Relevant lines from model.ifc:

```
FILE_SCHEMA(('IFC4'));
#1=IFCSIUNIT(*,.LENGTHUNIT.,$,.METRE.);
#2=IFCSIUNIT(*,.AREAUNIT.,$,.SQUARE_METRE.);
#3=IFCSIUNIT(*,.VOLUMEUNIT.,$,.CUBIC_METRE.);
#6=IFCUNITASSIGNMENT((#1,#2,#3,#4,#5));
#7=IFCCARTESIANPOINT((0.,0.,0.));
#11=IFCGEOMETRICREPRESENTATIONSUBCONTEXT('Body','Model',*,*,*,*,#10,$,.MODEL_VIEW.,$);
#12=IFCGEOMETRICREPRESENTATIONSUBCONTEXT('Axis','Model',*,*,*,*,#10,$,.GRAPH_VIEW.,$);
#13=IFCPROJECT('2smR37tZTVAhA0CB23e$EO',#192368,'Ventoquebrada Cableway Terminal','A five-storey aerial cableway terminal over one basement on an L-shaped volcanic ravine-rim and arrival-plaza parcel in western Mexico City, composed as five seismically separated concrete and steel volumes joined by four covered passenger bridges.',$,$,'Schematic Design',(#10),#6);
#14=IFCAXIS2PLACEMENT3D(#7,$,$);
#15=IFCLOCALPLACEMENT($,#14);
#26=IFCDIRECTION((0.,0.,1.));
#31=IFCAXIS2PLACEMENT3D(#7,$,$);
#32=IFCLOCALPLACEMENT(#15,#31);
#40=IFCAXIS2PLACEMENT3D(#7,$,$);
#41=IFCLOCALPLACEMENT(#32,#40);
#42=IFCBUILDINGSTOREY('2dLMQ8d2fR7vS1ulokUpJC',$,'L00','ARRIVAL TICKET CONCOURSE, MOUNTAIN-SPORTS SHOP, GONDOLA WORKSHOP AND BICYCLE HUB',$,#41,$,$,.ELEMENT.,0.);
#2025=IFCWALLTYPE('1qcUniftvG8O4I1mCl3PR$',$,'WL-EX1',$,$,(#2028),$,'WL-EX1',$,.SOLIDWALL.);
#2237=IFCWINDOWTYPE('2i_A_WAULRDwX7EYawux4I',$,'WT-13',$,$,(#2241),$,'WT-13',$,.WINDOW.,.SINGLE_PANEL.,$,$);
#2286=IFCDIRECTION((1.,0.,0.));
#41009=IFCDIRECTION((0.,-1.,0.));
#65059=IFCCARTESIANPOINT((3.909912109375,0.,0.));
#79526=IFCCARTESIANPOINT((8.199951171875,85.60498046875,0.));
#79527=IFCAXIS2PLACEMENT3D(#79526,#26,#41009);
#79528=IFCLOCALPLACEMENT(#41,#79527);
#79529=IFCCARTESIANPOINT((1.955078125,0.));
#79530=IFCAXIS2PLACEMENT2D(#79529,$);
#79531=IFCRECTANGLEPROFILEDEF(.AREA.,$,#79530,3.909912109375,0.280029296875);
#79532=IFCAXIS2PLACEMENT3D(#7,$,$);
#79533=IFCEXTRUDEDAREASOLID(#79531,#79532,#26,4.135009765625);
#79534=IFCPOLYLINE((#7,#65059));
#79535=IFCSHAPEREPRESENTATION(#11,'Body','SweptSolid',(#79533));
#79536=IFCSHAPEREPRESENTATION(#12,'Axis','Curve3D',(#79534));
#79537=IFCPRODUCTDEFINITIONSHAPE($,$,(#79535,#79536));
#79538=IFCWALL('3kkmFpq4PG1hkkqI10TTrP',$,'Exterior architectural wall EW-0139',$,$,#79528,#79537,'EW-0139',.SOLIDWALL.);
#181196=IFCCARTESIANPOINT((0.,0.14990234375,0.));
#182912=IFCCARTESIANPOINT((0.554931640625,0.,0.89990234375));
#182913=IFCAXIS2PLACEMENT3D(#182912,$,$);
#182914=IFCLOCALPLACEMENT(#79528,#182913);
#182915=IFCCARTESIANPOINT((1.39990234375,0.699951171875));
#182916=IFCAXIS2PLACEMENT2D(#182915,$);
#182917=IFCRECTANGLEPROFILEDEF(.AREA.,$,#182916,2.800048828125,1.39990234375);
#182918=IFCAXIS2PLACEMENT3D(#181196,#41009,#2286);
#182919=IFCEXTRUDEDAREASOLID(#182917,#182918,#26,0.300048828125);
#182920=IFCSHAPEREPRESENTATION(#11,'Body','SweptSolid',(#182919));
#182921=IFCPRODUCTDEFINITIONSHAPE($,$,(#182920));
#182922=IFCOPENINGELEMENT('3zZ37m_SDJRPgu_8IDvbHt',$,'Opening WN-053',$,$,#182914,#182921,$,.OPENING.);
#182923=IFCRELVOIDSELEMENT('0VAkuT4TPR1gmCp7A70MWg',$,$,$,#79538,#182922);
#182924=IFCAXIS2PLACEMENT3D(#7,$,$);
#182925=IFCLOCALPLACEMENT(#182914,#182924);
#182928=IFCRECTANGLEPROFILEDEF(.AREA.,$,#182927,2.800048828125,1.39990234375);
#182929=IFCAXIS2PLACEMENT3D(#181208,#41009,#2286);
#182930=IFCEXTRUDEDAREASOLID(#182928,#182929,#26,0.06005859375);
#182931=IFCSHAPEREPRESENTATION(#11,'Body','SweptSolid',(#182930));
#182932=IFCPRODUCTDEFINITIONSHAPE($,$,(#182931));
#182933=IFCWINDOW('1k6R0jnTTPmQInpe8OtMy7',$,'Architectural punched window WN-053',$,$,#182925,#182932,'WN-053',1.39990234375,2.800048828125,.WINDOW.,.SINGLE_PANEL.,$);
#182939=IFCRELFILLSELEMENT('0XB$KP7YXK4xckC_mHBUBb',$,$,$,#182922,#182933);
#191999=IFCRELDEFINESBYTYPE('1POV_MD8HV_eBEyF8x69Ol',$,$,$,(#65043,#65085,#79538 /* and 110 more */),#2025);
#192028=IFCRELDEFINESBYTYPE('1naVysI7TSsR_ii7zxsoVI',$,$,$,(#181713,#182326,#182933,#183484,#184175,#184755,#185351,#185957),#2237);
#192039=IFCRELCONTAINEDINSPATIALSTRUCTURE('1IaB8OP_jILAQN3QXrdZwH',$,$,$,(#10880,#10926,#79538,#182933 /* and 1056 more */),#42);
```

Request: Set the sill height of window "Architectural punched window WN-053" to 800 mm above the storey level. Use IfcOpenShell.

```python
import numpy as np
import ifcopenshell
import ifcopenshell.api.geometry
import ifcopenshell.geom
import ifcopenshell.util.element
import ifcopenshell.util.placement
import ifcopenshell.util.shape
import ifcopenshell.util.unit

model = ifcopenshell.open("model.ifc")
unit_scale = ifcopenshell.util.unit.calculate_unit_scale(model)

window = model.by_guid("1k6R0jnTTPmQInpe8OtMy7")
opening = window.FillsVoids[0].RelatingOpeningElement
storey = ifcopenshell.util.element.get_container(window, ifc_class="IfcBuildingStorey")
level = ifcopenshell.util.placement.get_local_placement(storey.ObjectPlacement)[2, 3]

# The opening's origin need not be at the sill, so measure its lowest point.
shape = ifcopenshell.geom.create_shape(ifcopenshell.geom.settings(), opening)
bottom = ifcopenshell.util.shape.get_shape_bottom_elevation(shape, shape.geometry) / unit_scale
dz = level + 0.8 / unit_scale - bottom

shift = np.array([0.0, 0.0, dz])
# The window is placed relative to its opening, so it follows when the opening moves.
matrix = ifcopenshell.util.placement.get_local_placement(opening.ObjectPlacement)
matrix[:3, 3] += shift
ifcopenshell.api.geometry.edit_object_placement(
    model, product=opening, matrix=matrix, is_si=False, should_transform_children=True
)

print(f"moved by {dz * unit_scale:+.3f} m")

model.write("model_updated.ifc")
```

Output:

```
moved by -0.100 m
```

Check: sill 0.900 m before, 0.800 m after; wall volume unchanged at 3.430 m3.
